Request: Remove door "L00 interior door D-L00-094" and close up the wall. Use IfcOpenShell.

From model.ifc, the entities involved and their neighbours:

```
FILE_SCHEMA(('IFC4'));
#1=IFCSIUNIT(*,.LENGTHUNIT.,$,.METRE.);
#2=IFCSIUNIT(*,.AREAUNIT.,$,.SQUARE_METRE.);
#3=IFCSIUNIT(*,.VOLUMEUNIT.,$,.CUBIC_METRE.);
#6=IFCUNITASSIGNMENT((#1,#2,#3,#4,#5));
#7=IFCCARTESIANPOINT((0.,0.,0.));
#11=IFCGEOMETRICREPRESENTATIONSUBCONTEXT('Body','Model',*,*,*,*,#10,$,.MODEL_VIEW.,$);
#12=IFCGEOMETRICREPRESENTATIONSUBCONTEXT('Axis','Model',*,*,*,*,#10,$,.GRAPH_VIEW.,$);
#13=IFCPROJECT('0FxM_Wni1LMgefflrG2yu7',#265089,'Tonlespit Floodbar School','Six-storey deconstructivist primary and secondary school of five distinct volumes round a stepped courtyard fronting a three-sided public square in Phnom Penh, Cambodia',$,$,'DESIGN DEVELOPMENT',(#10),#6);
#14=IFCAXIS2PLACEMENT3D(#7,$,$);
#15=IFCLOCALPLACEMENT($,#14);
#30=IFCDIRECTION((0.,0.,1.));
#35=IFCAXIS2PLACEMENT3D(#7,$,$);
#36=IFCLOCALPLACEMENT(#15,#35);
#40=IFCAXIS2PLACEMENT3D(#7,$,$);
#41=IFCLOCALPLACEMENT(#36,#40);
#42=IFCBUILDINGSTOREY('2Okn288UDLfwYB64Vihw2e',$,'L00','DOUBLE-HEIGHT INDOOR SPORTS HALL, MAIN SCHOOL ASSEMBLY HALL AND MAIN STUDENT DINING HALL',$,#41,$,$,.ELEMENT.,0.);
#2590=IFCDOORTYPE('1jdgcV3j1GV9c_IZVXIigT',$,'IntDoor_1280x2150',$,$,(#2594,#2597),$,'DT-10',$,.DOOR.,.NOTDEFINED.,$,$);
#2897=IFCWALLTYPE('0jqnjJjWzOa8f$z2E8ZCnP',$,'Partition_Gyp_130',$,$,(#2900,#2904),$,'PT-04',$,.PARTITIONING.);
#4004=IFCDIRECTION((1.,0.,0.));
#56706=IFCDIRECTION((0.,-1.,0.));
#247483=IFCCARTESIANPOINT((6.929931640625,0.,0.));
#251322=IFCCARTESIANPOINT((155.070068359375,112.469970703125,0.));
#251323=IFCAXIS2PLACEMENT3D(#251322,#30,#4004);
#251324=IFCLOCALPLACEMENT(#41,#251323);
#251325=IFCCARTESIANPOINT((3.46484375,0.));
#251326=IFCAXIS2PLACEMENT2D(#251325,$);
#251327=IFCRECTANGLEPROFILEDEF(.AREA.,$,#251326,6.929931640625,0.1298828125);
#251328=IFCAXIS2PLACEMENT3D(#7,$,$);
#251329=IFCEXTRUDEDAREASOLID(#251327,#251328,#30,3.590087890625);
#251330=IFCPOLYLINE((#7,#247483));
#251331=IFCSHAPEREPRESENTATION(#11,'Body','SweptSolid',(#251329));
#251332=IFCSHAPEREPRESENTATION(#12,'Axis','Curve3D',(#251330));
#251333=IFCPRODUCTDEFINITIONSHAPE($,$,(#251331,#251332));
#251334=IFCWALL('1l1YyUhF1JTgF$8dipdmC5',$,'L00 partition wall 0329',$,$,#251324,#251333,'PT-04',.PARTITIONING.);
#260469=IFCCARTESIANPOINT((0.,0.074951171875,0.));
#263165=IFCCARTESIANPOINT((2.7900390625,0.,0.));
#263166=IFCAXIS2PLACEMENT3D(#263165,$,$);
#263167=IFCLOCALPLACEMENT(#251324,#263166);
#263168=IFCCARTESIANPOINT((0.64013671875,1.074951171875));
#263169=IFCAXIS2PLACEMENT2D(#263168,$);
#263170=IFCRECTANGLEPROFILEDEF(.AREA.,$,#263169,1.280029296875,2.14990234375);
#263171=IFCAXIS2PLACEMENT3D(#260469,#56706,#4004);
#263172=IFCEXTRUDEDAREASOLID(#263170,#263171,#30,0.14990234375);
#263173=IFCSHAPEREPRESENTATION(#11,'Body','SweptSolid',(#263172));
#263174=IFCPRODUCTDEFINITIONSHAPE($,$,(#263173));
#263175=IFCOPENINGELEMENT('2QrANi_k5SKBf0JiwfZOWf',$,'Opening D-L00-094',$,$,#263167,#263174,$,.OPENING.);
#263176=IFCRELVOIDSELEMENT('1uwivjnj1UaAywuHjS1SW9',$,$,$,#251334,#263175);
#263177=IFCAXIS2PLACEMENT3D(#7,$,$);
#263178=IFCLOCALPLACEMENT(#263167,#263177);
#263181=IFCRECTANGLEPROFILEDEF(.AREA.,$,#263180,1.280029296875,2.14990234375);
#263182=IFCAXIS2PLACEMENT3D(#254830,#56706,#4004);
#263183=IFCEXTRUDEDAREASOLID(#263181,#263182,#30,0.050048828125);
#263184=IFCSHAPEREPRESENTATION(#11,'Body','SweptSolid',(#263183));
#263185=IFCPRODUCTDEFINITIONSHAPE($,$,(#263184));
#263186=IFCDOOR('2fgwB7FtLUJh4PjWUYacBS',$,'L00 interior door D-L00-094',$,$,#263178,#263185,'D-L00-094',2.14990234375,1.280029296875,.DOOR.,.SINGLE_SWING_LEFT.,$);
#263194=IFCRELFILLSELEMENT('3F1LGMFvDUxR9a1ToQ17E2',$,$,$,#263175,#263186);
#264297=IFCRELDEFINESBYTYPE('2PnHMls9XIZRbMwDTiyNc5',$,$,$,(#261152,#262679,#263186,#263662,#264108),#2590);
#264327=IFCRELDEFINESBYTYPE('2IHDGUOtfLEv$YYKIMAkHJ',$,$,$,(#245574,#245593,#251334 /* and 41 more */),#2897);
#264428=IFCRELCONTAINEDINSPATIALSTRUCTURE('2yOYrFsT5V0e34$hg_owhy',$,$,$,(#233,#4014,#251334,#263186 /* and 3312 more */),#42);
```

```python
import ifcopenshell
import ifcopenshell.api.feature
import ifcopenshell.api.root
import ifcopenshell.geom
import ifcopenshell.util.shape

model = ifcopenshell.open("model.ifc")
settings = ifcopenshell.geom.settings()


def volume(element):
    """Net volume in cubic metres, openings subtracted."""
    shape = ifcopenshell.geom.create_shape(settings, element)
    return ifcopenshell.util.shape.get_volume(shape.geometry)


door = model.by_id(263186)
opening = door.FillsVoids[0].RelatingOpeningElement
wall = opening.VoidsElements[0].RelatingBuildingElement
before = volume(wall)

ifcopenshell.api.root.remove_product(model, product=door)
ifcopenshell.api.feature.remove_feature(model, feature=opening)

after = volume(wall)

print(f"wall volume {before:.3f} -> {after:.3f} m3")

model.write("model_v2.ifc")
```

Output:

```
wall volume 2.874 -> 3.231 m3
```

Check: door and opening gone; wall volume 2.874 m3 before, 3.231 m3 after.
